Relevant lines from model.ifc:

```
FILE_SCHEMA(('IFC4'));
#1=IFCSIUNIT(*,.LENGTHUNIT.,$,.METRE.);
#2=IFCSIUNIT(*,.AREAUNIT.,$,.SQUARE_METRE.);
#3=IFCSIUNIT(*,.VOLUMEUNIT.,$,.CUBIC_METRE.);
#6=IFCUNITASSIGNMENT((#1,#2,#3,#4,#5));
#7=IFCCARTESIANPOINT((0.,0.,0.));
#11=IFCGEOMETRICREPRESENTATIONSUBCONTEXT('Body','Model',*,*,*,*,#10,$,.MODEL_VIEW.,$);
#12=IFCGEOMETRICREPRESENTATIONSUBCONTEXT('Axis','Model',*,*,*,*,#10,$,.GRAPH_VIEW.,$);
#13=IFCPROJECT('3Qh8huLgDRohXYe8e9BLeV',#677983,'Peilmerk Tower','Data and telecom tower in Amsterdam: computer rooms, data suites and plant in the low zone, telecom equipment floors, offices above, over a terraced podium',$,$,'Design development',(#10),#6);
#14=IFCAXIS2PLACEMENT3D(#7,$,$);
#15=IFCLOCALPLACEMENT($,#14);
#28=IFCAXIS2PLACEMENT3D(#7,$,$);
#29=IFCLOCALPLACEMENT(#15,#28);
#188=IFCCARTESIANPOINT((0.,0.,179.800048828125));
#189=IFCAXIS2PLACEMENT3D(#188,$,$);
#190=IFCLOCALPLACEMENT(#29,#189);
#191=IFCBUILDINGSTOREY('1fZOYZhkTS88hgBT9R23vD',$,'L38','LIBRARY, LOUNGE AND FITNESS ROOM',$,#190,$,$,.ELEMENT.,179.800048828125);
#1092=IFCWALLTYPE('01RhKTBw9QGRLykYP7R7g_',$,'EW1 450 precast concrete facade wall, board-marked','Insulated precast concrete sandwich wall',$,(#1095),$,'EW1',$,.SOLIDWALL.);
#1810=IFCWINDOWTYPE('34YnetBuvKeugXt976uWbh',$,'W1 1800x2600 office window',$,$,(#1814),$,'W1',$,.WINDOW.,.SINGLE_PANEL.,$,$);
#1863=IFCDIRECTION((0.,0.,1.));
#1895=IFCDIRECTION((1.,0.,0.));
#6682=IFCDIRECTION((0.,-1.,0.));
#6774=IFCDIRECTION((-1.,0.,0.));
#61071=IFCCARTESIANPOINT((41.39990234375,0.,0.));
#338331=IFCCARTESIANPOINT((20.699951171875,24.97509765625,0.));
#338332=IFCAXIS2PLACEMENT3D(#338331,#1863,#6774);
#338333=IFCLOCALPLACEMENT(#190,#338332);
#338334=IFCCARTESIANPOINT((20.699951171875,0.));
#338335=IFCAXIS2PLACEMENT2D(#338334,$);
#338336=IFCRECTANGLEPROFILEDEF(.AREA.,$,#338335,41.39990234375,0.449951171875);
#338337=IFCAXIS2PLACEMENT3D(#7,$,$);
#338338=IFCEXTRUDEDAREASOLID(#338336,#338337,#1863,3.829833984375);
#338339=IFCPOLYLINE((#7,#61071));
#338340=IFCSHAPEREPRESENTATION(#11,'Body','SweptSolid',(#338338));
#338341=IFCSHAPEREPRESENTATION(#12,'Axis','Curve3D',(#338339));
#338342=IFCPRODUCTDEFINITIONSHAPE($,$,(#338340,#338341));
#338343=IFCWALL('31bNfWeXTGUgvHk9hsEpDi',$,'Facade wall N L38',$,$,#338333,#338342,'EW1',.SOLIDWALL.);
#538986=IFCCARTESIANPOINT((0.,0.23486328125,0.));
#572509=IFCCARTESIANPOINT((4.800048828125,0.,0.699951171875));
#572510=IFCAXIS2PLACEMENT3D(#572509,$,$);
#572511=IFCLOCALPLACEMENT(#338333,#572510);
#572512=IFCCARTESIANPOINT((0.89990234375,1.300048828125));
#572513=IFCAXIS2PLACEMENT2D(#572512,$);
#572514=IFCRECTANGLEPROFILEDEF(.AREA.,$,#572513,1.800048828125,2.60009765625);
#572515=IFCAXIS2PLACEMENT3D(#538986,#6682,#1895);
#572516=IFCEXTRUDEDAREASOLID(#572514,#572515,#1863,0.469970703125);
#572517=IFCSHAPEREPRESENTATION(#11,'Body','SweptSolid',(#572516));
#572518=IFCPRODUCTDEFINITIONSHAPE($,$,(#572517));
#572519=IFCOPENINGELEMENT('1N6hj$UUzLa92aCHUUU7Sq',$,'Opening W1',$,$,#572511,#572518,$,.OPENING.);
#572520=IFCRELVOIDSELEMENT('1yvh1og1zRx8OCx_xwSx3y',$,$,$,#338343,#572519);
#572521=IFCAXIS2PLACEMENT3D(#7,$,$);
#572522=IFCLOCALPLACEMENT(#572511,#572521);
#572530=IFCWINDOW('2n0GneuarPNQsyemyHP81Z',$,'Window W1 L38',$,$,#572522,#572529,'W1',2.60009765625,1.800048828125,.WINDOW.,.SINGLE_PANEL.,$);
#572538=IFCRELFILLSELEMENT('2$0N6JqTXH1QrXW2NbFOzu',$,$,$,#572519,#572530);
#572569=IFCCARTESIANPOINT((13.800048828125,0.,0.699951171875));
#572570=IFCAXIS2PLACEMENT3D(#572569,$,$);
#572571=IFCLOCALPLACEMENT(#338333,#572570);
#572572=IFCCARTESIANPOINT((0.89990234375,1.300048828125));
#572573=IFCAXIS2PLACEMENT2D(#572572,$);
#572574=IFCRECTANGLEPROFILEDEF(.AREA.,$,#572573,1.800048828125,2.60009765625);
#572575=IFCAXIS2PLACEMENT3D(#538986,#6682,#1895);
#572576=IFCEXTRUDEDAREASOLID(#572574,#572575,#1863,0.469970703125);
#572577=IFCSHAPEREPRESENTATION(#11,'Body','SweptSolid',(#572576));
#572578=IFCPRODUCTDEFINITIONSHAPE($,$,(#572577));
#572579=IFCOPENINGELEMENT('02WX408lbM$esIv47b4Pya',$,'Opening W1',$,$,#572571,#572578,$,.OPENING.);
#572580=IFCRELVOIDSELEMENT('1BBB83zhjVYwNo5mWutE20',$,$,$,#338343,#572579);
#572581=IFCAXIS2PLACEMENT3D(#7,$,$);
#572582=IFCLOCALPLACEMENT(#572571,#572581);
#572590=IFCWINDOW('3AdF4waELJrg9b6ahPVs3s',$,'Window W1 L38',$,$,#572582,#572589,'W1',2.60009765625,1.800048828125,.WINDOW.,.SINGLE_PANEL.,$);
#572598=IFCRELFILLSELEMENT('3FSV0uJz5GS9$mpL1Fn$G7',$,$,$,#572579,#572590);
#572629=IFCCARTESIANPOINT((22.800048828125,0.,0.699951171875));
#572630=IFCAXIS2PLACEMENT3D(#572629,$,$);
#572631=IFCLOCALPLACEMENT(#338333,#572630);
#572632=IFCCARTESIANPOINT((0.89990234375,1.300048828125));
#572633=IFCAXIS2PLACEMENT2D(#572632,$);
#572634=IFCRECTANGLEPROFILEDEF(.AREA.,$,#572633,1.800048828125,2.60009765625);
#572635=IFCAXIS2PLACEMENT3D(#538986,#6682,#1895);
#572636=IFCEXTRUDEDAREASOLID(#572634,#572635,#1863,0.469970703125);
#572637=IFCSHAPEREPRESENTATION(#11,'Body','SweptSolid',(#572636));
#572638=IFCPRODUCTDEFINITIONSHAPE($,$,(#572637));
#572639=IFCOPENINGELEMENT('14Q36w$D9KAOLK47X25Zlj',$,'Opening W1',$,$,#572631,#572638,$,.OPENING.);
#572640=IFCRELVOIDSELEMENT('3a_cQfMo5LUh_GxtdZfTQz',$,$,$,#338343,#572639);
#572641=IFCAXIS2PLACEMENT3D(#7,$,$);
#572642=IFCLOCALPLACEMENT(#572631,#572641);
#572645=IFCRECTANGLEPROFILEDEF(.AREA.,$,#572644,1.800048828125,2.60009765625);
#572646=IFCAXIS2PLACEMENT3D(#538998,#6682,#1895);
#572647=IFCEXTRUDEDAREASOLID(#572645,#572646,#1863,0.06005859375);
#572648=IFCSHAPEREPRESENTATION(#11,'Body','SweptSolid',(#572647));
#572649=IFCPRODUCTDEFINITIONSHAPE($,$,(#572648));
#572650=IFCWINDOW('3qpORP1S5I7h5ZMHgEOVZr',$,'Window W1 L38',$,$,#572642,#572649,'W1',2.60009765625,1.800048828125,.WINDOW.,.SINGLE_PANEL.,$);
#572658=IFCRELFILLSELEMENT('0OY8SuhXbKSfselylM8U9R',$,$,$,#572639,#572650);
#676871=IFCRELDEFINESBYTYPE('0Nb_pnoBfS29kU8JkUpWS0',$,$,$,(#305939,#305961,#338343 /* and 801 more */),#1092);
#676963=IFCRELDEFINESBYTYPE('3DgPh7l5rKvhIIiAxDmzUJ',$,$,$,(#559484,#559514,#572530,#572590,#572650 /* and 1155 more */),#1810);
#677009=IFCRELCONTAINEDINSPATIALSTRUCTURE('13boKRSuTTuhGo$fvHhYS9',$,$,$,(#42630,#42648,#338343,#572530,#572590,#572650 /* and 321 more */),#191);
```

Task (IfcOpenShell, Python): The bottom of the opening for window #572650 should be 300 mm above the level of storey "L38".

```python
import numpy as np
import ifcopenshell
import ifcopenshell.api.geometry
import ifcopenshell.geom
import ifcopenshell.util.element
import ifcopenshell.util.placement
import ifcopenshell.util.shape
import ifcopenshell.util.unit

model = ifcopenshell.open("model.ifc")
unit_scale = ifcopenshell.util.unit.calculate_unit_scale(model)

window = model.by_guid("3qpORP1S5I7h5ZMHgEOVZr")
opening = window.FillsVoids[0].RelatingOpeningElement
storey = ifcopenshell.util.element.get_container(window, ifc_class="IfcBuildingStorey")
level = ifcopenshell.util.placement.get_local_placement(storey.ObjectPlacement)[2, 3]

# The opening's origin need not be at the sill, so measure its lowest point.
shape = ifcopenshell.geom.create_shape(ifcopenshell.geom.settings(), opening)
bottom = ifcopenshell.util.shape.get_shape_bottom_elevation(shape, shape.geometry) / unit_scale
dz = level + 0.3 / unit_scale - bottom

shift = np.array([0.0, 0.0, dz])
# The window is placed relative to its opening, so it follows when the opening moves.
matrix = ifcopenshell.util.placement.get_local_placement(opening.ObjectPlacement)
matrix[:3, 3] += shift
ifcopenshell.api.geometry.edit_object_placement(
    model, product=opening, matrix=matrix, is_si=False, should_transform_children=True
)

print(f"moved by {dz * unit_scale:+.3f} m")

model.write("model-out.ifc")
```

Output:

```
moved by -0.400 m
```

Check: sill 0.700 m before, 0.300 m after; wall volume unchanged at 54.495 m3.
